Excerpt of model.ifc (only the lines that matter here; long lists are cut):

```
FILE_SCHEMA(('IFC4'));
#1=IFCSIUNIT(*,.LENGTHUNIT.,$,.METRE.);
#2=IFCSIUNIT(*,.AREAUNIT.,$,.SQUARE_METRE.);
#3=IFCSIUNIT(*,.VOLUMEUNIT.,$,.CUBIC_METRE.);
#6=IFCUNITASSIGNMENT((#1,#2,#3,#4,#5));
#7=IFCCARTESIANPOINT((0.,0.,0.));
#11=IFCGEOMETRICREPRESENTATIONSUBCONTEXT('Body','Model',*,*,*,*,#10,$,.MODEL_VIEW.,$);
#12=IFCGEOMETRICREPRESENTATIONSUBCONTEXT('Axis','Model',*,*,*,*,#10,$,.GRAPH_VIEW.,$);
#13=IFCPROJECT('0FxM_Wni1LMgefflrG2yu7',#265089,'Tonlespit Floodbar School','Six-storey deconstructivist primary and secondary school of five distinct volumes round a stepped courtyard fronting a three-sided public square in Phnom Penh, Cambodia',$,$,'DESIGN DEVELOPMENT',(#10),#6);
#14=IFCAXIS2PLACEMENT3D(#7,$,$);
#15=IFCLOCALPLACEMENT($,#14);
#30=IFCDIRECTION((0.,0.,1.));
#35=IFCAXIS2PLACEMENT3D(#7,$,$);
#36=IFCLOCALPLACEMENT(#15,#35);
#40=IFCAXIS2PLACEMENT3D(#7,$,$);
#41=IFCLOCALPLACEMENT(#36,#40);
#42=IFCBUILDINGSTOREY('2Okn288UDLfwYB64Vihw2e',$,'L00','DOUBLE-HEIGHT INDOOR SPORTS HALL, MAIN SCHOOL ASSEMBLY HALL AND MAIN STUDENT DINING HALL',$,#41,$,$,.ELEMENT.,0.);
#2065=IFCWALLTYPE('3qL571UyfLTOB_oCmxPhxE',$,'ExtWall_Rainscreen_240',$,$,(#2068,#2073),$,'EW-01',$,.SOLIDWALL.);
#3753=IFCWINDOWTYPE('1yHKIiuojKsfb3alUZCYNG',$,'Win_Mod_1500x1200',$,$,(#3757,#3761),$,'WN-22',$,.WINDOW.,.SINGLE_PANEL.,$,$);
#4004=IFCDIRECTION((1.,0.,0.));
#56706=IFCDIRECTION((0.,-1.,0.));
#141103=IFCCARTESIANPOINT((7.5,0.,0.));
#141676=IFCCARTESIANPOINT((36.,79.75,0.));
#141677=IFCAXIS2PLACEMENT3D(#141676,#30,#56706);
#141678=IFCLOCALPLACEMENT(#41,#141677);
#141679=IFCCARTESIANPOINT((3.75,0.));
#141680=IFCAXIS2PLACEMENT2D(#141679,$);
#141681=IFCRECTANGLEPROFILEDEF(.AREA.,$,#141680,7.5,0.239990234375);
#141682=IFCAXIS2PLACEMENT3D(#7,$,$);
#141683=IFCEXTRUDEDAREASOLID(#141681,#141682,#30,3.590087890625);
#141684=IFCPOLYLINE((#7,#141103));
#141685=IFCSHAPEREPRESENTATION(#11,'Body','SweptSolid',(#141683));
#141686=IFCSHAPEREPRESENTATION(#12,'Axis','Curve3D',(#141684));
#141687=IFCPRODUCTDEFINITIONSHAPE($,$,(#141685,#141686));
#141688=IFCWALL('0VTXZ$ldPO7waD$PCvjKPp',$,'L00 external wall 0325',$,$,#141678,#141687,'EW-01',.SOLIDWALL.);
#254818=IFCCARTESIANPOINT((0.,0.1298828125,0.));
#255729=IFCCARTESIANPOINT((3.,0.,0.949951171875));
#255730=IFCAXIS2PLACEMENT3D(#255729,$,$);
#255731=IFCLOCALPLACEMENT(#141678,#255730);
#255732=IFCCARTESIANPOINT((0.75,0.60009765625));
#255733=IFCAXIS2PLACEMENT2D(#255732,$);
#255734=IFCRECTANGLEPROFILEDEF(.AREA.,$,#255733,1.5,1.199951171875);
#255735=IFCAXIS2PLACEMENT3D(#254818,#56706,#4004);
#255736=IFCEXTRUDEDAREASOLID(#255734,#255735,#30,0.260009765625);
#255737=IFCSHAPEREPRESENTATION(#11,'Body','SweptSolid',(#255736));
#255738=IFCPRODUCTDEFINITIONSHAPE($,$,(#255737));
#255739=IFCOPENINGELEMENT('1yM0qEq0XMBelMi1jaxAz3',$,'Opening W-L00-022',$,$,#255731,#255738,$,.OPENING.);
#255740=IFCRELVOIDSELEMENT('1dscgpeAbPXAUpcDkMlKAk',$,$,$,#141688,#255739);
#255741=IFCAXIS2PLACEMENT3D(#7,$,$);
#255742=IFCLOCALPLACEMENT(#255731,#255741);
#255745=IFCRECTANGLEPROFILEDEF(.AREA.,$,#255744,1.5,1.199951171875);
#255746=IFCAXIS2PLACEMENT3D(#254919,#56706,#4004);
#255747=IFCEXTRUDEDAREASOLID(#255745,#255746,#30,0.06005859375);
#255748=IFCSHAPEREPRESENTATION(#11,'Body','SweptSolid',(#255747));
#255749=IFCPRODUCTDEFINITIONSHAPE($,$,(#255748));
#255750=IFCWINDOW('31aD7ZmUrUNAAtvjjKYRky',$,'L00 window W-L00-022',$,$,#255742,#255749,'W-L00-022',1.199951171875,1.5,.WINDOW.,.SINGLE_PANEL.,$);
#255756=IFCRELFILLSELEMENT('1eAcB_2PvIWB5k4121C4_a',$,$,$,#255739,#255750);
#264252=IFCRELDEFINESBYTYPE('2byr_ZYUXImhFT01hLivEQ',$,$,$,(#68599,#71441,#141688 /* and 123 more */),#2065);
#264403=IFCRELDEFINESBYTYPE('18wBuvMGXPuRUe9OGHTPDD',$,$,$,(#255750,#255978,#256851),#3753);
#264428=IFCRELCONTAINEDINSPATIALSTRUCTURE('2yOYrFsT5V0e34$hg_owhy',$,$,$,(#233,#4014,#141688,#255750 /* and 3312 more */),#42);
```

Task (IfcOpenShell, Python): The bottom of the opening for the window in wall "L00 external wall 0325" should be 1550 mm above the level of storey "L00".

```python
import numpy as np
import ifcopenshell
import ifcopenshell.api.geometry
import ifcopenshell.geom
import ifcopenshell.util.element
import ifcopenshell.util.placement
import ifcopenshell.util.shape
import ifcopenshell.util.unit

model = ifcopenshell.open("model.ifc")
unit_scale = ifcopenshell.util.unit.calculate_unit_scale(model)

window = model.by_guid("31aD7ZmUrUNAAtvjjKYRky")
opening = window.FillsVoids[0].RelatingOpeningElement
storey = ifcopenshell.util.element.get_container(window, ifc_class="IfcBuildingStorey")
level = ifcopenshell.util.placement.get_local_placement(storey.ObjectPlacement)[2, 3]

# The opening's origin need not be at the sill, so measure its lowest point.
shape = ifcopenshell.geom.create_shape(ifcopenshell.geom.settings(), opening)
bottom = ifcopenshell.util.shape.get_shape_bottom_elevation(shape, shape.geometry) / unit_scale
dz = level + 1.55 / unit_scale - bottom

shift = np.array([0.0, 0.0, dz])
# The window is placed relative to its opening, so it follows when the opening moves.
matrix = ifcopenshell.util.placement.get_local_placement(opening.ObjectPlacement)
matrix[:3, 3] += shift
ifcopenshell.api.geometry.edit_object_placement(
    model, product=opening, matrix=matrix, is_si=False, should_transform_children=True
)

print(f"moved by {dz * unit_scale:+.3f} m")

model.write("model_rev.ifc")
```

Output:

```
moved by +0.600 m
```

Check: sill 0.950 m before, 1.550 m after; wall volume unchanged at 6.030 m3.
